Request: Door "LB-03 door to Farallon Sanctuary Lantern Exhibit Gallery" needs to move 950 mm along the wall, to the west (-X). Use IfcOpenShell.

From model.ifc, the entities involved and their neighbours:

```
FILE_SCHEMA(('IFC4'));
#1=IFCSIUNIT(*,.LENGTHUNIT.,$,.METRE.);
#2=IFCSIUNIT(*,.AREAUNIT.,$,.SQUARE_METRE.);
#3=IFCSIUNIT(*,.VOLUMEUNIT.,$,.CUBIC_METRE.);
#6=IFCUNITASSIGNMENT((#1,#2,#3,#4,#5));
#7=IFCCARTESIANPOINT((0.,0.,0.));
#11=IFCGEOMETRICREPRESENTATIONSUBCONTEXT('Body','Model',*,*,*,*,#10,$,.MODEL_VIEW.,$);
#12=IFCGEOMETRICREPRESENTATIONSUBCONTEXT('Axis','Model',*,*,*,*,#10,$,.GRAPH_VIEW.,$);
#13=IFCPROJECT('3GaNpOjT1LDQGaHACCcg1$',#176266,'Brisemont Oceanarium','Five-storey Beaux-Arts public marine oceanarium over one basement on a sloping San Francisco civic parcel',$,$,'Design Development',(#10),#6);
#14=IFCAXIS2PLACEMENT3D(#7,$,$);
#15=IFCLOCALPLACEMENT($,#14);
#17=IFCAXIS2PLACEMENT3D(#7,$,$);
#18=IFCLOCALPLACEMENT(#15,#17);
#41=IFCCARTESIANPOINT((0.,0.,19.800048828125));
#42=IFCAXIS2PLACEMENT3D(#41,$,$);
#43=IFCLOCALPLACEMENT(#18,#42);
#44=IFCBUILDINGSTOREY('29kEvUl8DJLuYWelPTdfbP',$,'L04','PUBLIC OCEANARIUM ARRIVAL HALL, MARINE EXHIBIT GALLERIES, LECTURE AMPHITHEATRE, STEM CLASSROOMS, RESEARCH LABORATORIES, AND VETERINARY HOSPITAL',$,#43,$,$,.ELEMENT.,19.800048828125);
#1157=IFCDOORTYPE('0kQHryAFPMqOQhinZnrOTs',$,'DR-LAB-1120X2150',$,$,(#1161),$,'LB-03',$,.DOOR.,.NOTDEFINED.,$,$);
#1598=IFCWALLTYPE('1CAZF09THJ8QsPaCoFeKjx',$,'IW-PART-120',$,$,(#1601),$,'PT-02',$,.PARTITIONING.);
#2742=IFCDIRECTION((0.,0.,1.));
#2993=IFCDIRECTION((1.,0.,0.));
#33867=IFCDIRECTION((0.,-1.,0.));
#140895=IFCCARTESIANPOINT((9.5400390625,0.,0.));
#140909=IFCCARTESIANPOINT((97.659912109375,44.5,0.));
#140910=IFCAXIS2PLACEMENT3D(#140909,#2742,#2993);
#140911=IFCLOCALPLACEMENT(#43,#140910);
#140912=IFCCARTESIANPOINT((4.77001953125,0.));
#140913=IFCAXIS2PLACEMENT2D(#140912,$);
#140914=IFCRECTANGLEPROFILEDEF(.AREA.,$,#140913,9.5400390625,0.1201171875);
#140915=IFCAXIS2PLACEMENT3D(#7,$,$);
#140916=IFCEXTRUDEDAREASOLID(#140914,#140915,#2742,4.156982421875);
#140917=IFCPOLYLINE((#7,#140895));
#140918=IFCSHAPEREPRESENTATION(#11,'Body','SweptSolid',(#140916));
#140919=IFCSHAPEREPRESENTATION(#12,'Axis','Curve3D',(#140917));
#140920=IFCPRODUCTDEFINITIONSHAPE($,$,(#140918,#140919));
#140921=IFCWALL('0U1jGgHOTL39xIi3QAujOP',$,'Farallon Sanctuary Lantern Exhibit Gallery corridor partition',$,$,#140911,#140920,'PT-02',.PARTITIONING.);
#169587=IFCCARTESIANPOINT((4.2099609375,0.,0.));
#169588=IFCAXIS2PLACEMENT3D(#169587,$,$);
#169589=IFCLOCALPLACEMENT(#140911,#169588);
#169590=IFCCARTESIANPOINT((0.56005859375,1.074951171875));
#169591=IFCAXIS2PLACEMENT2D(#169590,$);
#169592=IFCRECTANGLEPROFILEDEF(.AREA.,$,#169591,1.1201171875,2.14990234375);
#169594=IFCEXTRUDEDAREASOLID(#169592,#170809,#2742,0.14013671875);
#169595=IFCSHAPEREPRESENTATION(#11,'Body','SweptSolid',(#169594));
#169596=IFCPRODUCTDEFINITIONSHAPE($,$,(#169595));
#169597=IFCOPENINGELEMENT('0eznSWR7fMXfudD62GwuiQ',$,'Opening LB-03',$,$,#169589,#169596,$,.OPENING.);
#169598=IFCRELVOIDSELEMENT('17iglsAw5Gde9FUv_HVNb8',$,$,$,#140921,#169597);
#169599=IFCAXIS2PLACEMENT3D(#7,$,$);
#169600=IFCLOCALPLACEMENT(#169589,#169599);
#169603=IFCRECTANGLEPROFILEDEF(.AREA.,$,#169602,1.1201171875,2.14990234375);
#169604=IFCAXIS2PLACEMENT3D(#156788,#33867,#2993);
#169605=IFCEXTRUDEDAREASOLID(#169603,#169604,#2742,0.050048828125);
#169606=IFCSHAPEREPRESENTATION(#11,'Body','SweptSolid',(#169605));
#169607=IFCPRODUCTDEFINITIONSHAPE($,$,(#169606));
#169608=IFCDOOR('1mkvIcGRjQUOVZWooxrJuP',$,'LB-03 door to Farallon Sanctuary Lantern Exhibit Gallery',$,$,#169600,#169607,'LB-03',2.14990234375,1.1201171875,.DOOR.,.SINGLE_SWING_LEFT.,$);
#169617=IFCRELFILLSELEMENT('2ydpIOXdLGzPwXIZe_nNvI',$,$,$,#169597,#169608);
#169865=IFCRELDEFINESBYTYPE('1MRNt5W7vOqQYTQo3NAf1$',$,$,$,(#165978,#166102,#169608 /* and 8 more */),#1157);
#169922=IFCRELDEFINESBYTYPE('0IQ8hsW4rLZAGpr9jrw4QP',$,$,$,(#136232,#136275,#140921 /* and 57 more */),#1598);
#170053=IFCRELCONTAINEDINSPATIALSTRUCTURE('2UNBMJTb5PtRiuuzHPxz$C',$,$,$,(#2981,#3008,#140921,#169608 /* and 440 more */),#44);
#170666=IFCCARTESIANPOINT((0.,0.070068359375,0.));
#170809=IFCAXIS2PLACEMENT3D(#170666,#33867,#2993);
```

```python
import ifcopenshell
import ifcopenshell.api.geometry
import ifcopenshell.util.placement
import ifcopenshell.util.unit

model = ifcopenshell.open("model.ifc")
unit_scale = ifcopenshell.util.unit.calculate_unit_scale(model)

door = model.by_guid("1mkvIcGRjQUOVZWooxrJuP")
opening = door.FillsVoids[0].RelatingOpeningElement
wall = opening.VoidsElements[0].RelatingBuildingElement

wall_matrix = ifcopenshell.util.placement.get_local_placement(wall.ObjectPlacement)
shift = wall_matrix[:3, 0] * -0.95 / unit_scale
before = ifcopenshell.util.placement.get_local_placement(door.ObjectPlacement)[:3, 3].copy()

# The door is placed relative to its opening, so it follows when the opening moves.
matrix = ifcopenshell.util.placement.get_local_placement(opening.ObjectPlacement)
matrix[:3, 3] += shift
ifcopenshell.api.geometry.edit_object_placement(
    model, product=opening, matrix=matrix, is_si=False, should_transform_children=True
)

after = ifcopenshell.util.placement.get_local_placement(door.ObjectPlacement)[:3, 3]
print("door moved by", (after - before).round(3) + 0.0)

model.write("model_rev.ifc")
```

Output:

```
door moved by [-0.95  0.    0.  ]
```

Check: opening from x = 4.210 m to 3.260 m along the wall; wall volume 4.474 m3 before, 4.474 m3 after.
